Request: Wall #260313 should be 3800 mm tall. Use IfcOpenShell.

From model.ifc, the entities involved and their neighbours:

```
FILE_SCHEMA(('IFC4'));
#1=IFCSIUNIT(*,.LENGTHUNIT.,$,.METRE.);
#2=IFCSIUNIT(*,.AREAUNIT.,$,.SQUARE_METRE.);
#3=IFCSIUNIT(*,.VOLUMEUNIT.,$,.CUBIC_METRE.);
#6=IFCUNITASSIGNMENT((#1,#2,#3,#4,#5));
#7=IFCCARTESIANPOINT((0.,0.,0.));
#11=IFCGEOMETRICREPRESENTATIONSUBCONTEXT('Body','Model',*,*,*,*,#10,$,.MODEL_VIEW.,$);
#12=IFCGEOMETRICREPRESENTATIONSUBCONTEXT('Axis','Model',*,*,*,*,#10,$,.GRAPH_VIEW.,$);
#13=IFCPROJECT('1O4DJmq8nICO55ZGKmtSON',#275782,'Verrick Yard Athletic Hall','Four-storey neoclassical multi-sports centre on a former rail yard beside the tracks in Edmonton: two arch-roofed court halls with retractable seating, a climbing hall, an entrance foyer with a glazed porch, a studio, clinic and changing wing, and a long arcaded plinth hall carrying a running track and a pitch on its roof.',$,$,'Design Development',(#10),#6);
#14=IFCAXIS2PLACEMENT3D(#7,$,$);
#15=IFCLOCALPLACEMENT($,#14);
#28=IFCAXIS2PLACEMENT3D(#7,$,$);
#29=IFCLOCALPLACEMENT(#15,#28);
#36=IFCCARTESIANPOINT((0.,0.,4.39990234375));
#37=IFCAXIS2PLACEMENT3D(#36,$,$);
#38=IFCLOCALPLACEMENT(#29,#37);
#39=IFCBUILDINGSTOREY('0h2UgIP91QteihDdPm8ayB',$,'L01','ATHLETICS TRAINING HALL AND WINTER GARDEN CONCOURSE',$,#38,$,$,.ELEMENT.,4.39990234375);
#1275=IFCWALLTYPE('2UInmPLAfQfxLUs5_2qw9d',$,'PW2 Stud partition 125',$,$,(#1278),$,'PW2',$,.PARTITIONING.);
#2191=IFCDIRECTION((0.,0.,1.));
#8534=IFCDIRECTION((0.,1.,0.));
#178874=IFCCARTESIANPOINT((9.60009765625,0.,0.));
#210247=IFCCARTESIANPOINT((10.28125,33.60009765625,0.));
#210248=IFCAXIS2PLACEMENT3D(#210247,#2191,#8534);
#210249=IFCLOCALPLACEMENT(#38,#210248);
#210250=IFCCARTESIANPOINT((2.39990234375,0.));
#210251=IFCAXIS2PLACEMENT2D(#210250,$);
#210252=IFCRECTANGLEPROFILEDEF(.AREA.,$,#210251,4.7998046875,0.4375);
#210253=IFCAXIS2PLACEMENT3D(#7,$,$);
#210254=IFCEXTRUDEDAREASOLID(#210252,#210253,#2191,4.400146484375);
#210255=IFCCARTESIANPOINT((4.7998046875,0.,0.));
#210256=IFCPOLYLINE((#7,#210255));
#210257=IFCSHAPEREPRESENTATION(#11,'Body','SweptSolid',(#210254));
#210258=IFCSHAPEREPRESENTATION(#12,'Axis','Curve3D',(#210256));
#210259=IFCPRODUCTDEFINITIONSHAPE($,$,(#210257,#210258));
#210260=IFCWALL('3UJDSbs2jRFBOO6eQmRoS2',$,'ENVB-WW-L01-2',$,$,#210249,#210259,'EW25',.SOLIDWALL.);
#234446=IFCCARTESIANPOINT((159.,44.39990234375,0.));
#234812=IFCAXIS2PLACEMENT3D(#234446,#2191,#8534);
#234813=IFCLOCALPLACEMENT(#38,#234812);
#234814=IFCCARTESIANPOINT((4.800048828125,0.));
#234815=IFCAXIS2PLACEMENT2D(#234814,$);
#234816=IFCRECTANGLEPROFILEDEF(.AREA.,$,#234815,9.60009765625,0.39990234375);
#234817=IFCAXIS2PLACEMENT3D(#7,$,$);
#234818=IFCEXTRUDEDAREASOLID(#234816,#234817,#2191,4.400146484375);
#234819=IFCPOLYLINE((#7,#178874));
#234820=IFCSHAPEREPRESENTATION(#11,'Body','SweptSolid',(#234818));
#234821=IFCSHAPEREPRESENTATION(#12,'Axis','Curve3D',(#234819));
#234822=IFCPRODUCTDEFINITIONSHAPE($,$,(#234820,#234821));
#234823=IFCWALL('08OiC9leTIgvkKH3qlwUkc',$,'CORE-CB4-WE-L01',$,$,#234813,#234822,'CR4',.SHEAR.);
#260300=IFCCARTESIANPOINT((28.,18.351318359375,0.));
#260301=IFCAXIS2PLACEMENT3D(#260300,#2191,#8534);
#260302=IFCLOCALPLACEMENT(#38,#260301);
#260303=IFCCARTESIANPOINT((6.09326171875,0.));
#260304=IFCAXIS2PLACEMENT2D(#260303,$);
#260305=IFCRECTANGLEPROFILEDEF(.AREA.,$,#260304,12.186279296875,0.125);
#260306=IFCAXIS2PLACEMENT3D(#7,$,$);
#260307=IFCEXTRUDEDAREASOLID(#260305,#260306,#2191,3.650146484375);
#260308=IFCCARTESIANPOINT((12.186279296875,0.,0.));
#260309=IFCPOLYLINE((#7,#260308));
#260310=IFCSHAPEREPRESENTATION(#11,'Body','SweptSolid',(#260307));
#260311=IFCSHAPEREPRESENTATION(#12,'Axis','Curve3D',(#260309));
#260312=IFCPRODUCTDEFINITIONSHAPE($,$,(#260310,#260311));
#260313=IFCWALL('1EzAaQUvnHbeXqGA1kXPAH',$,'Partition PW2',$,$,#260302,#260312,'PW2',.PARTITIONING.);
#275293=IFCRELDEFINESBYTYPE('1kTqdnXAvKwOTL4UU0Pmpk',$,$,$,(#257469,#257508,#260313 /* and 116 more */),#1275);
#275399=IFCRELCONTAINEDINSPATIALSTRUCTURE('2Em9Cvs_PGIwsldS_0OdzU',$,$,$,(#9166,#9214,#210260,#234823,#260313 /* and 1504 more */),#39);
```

```python
import ifcopenshell
import ifcopenshell.geom
import ifcopenshell.util.representation
import ifcopenshell.util.shape

model = ifcopenshell.open("model.ifc")
settings = ifcopenshell.geom.settings()


def volume(element):
    """Net volume in cubic metres, openings subtracted."""
    shape = ifcopenshell.geom.create_shape(settings, element)
    return ifcopenshell.util.shape.get_volume(shape.geometry)


wall = model.by_guid("1EzAaQUvnHbeXqGA1kXPAH")
before = volume(wall)

body = ifcopenshell.util.representation.get_representation(wall, "Model", "Body")
solid = body.Items[0]
old_height = solid.Depth
solid.Depth = 3.8
after = volume(wall)

print(f"height {old_height:g} -> {solid.Depth:g}, volume {before:.3f} -> {after:.3f} m3")

model.write("model_edited.ifc")
```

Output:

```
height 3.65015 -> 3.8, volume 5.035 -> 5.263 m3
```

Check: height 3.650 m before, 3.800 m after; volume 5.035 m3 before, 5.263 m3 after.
